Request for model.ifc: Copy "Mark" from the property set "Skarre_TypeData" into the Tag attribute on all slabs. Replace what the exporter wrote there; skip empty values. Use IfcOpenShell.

First a look at what the model holds.

```python
import ifcopenshell
import ifcopenshell.util.element

model = ifcopenshell.open("model.ifc")
print(model.schema)
slabs = model.by_type("IfcSlab")
print(len(slabs), "slabs")
for e in slabs[:8]:
    source = ifcopenshell.util.element.get_pset(e, "Skarre_TypeData", "Mark")
    target = e.Tag
    print(e.id(), repr(source), repr(target), sep=" | ")
```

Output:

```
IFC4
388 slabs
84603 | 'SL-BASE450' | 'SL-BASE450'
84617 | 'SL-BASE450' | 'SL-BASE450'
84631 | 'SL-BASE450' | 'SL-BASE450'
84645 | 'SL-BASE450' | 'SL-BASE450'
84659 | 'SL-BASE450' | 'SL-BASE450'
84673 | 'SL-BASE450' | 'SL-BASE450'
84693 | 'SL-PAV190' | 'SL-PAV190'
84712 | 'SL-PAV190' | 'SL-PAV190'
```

```python
import ifcopenshell
import ifcopenshell.util.element

model = ifcopenshell.open("model.ifc")

count = 0
for e in model.by_type("IfcSlab"):
    value = ifcopenshell.util.element.get_pset(e, "Skarre_TypeData", "Mark")
    current = e.Tag
    if not value or not value.strip() or current == value:
        continue
    e.Tag = value
    count += 1

print(count, "slabs updated")

model.write("model_edited.ifc")
```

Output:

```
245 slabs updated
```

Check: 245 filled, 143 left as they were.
